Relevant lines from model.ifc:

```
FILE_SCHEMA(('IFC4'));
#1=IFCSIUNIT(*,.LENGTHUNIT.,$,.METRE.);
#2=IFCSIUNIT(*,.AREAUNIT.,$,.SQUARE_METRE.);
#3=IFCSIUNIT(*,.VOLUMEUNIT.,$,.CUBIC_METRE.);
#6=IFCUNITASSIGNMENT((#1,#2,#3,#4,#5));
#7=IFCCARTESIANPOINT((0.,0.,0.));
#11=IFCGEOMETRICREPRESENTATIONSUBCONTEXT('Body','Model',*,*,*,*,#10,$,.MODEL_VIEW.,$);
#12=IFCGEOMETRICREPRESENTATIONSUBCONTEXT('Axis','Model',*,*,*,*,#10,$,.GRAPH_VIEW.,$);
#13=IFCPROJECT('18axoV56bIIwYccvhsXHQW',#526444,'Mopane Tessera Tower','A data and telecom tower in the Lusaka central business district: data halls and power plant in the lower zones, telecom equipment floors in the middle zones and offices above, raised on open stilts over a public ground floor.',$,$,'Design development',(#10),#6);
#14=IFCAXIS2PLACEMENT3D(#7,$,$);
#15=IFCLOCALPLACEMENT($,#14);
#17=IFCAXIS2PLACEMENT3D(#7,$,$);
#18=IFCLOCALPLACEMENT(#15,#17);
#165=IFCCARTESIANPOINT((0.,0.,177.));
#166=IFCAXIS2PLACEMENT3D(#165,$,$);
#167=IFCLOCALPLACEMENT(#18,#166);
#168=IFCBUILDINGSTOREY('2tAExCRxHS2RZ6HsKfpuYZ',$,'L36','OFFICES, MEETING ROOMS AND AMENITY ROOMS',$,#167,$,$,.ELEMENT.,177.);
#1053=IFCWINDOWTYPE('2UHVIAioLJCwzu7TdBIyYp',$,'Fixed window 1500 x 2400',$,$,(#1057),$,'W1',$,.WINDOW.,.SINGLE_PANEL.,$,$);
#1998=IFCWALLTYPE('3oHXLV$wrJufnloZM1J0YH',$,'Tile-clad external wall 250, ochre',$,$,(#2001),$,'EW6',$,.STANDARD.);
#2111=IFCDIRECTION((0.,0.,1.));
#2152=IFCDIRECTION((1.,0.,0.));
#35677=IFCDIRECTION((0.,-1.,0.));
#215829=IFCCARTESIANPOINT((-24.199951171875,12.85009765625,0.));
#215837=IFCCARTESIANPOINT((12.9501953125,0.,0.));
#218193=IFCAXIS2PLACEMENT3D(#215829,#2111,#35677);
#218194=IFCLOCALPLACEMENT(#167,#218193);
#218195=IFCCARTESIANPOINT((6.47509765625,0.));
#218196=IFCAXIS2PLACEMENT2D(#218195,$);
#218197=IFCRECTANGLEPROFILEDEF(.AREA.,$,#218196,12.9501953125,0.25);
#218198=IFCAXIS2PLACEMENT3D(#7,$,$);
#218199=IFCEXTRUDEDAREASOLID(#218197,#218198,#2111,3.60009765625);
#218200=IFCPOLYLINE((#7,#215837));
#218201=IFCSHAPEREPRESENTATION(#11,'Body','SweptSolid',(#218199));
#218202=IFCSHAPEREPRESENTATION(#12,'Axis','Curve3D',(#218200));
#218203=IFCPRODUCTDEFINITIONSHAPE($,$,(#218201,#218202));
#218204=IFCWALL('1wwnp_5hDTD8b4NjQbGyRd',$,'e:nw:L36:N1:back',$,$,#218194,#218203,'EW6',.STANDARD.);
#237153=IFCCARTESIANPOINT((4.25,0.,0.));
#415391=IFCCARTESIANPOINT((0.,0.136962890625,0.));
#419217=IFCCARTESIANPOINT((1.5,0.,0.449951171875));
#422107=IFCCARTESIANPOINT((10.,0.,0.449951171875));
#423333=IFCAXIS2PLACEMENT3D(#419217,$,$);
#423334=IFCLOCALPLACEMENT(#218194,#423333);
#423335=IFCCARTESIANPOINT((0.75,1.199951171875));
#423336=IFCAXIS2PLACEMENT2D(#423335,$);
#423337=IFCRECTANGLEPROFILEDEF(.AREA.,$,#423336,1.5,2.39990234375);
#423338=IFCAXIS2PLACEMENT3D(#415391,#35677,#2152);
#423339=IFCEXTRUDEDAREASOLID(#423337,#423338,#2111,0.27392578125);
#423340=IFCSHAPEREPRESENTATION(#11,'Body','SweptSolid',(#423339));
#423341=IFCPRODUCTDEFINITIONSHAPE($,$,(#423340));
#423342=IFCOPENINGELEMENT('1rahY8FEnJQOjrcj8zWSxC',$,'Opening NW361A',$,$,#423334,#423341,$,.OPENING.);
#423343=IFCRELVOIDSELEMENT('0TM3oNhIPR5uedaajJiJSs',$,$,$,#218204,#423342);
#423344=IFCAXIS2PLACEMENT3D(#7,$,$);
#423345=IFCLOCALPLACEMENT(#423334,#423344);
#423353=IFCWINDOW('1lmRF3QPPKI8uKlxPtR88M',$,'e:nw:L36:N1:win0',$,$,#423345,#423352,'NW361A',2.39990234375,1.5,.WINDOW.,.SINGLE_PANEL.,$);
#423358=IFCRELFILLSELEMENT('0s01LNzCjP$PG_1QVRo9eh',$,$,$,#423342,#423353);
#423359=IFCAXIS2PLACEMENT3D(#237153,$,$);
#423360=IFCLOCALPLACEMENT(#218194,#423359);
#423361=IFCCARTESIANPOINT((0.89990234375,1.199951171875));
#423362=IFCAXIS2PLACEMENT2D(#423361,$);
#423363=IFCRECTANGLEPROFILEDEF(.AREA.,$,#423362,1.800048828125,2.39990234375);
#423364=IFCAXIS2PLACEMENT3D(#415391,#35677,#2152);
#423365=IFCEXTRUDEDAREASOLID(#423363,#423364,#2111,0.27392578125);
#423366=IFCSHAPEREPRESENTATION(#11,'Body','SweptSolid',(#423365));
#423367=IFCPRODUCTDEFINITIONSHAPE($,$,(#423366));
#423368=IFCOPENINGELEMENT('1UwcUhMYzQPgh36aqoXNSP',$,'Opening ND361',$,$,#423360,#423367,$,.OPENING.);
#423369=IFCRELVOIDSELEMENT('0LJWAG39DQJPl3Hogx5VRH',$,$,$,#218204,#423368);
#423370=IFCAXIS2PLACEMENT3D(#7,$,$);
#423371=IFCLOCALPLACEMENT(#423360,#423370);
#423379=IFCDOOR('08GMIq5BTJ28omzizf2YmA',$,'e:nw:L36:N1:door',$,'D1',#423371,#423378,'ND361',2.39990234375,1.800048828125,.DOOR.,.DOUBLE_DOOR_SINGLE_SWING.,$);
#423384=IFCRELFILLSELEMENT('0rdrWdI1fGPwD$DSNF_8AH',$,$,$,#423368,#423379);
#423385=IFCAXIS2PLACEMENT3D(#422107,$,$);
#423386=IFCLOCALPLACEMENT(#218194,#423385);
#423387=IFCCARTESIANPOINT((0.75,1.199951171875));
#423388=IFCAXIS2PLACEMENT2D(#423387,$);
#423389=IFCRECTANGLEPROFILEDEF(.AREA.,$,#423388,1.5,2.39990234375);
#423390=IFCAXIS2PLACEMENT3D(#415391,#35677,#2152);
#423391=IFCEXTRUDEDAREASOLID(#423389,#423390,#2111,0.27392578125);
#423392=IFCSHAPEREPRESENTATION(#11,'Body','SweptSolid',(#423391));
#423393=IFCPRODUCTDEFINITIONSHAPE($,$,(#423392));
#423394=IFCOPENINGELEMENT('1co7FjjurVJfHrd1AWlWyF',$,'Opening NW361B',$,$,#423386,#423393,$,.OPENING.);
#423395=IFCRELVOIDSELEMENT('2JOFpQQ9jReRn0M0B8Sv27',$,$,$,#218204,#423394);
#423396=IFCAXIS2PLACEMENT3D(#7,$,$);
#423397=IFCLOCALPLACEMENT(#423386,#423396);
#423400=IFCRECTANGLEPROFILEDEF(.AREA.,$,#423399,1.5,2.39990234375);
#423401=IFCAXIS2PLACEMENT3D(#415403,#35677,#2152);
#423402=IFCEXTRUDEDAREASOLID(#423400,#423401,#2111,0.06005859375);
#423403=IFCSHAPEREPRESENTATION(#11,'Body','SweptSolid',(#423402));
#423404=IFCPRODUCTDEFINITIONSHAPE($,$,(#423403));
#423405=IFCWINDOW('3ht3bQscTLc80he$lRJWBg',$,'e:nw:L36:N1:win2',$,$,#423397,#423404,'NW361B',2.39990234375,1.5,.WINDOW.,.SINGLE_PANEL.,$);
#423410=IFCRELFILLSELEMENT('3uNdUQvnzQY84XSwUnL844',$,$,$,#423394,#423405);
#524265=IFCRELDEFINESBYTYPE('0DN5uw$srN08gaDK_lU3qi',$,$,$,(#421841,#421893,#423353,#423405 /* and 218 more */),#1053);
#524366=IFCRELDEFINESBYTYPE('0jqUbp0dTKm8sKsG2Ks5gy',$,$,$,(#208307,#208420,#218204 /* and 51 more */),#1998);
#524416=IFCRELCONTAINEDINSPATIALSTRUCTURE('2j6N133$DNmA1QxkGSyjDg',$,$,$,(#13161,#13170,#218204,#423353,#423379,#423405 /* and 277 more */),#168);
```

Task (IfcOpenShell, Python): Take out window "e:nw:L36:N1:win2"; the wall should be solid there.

```python
import ifcopenshell
import ifcopenshell.api.feature
import ifcopenshell.api.root
import ifcopenshell.geom
import ifcopenshell.util.shape

model = ifcopenshell.open("model.ifc")
settings = ifcopenshell.geom.settings()


def volume(element):
    """Net volume in cubic metres, openings subtracted."""
    shape = ifcopenshell.geom.create_shape(settings, element)
    return ifcopenshell.util.shape.get_volume(shape.geometry)


window = model.by_guid("3ht3bQscTLc80he$lRJWBg")
opening = window.FillsVoids[0].RelatingOpeningElement
wall = opening.VoidsElements[0].RelatingBuildingElement
before = volume(wall)

ifcopenshell.api.root.remove_product(model, product=window)
ifcopenshell.api.feature.remove_feature(model, feature=opening)

after = volume(wall)

print(f"wall volume {before:.3f} -> {after:.3f} m3")

model.write("model_edited.ifc")
```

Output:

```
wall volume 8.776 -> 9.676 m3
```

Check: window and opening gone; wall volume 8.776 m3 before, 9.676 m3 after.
